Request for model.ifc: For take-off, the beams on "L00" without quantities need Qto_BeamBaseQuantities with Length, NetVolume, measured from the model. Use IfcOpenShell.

First a look at what the model holds.

```python
import ifcopenshell
import ifcopenshell.util.element
import ifcopenshell.util.unit

model = ifcopenshell.open("model.ifc")
print(model.schema)
for unit_type in ("LENGTHUNIT", "AREAUNIT", "VOLUMEUNIT"):
    print(unit_type, ifcopenshell.util.unit.calculate_unit_scale(model, unit_type))
storey = next(s for s in model.by_type("IfcBuildingStorey") if s.Name == "L00")
beams = [e for e in ifcopenshell.util.element.get_decomposition(storey) if e.is_a("IfcBeam")]
for e in sorted(beams, key=lambda e: e.id()):
    print(e.id(), e.is_a(), e.Name, list(ifcopenshell.util.element.get_psets(e, qtos_only=True)), sep=" | ")
```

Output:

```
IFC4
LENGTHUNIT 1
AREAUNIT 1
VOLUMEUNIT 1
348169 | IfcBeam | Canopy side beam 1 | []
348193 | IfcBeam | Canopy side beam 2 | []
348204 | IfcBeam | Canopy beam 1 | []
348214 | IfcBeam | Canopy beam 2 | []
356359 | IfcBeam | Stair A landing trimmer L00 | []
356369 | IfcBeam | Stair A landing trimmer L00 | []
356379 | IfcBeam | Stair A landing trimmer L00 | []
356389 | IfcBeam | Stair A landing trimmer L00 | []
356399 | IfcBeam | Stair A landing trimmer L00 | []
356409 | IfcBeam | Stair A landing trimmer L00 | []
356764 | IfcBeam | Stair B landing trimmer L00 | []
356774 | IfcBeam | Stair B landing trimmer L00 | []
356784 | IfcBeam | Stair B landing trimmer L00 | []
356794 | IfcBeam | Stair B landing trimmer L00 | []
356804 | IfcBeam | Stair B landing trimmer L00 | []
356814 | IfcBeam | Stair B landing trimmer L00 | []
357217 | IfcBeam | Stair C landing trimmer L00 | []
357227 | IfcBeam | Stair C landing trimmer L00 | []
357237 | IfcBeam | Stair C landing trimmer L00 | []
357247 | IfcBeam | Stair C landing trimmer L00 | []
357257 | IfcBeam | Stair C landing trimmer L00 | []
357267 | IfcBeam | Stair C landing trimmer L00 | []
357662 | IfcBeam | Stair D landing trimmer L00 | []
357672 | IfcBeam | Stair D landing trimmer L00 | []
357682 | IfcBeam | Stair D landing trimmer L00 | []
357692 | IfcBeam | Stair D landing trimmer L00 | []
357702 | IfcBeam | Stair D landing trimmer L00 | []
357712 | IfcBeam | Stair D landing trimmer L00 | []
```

```python
import ifcopenshell
import ifcopenshell.api.pset
import ifcopenshell.geom
import ifcopenshell.util.element
import ifcopenshell.util.shape
import ifcopenshell.util.unit

model = ifcopenshell.open("model.ifc")
unit_scale = ifcopenshell.util.unit.calculate_unit_scale(model)
volume_scale = ifcopenshell.util.unit.calculate_unit_scale(model, "VOLUMEUNIT")
settings = ifcopenshell.geom.settings()

storey = next(s for s in model.by_type("IfcBuildingStorey") if s.Name == "L00")
beams = [e for e in ifcopenshell.util.element.get_decomposition(storey) if e.is_a("IfcBeam")]

for e in sorted(beams, key=lambda e: e.id()):
    if ifcopenshell.util.element.get_psets(e, qtos_only=True, should_inherit=False):
        continue
    # Geometry comes back in metres, in the element's own axes.
    shape = ifcopenshell.geom.create_shape(settings, e)
    values = {
        "Length": ifcopenshell.util.shape.get_max_xyz(shape.geometry) / unit_scale,
        "NetVolume": ifcopenshell.util.shape.get_volume(shape.geometry) / volume_scale,
    }
    qto = ifcopenshell.api.pset.add_qto(model, product=e, name="Qto_BeamBaseQuantities")
    ifcopenshell.api.pset.edit_qto(model, qto=qto, properties=values)
    print(e.id(), {k: round(v, 3) for k, v in values.items()})

model.write("model_updated.ifc")
```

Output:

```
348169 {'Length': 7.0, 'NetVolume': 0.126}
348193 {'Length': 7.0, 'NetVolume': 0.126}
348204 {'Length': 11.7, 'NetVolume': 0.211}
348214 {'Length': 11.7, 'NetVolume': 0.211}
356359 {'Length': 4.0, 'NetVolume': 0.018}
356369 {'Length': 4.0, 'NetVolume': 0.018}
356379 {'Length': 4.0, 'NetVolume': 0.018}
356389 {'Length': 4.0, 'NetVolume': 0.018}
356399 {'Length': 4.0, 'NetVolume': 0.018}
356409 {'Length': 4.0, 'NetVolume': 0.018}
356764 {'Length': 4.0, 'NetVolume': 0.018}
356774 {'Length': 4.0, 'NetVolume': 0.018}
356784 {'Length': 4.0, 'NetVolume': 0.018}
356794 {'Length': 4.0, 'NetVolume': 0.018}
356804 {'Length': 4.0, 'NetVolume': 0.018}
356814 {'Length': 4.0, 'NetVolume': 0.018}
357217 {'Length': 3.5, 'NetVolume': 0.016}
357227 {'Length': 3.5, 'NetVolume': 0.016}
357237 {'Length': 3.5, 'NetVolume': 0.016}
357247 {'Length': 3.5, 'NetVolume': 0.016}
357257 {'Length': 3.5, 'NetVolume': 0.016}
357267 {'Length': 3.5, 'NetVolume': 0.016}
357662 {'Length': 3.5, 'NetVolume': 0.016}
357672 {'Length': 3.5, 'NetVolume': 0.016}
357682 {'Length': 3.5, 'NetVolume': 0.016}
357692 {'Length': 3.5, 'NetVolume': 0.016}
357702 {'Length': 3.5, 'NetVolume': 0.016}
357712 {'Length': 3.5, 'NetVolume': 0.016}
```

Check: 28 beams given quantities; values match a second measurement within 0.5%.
